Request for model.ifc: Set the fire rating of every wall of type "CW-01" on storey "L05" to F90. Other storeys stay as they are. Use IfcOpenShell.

First a look at what the model holds.

```python
import ifcopenshell
import ifcopenshell.util.element

model = ifcopenshell.open("model.ifc")
print(model.schema)
storey = next(s for s in model.by_type("IfcBuildingStorey") if s.Name == "L05")
walls = [e for e in ifcopenshell.util.element.get_decomposition(storey) if e.is_a("IfcWall")]
seen = {}
for e in walls:
    element_type = ifcopenshell.util.element.get_type(e)
    key = (element_type.Name if element_type != e and element_type else None, ifcopenshell.util.element.get_pset(e, "Pset_WallCommon", "FireRating"))
    seen[key] = seen.get(key, 0) + 1
for (name, value), count in sorted(seen.items(), key=str):
    print(count, "x", name, "|", value)
```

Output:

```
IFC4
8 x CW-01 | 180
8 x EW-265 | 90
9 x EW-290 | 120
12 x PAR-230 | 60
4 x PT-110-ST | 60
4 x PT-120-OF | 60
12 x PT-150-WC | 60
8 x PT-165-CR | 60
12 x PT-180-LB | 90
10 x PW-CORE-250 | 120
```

```python
import ifcopenshell
import ifcopenshell.api.pset
import ifcopenshell.util.element

model = ifcopenshell.open("model.ifc")

storey = next(s for s in model.by_type("IfcBuildingStorey") if s.Name == "L05")
walls = [e for e in ifcopenshell.util.element.get_decomposition(storey) if e.is_a("IfcWall")]

count = 0
for e in walls:
    element_type = ifcopenshell.util.element.get_type(e)
    if element_type in (None, e) or element_type.Name != "CW-01":
        continue
    # add_pset returns the element's existing set when there is one.
    pset = ifcopenshell.api.pset.add_pset(model, product=e, name="Pset_WallCommon")
    ifcopenshell.api.pset.edit_pset(model, pset=pset, properties={"FireRating": "F90"})
    count += 1

print(count, "walls updated")

model.write("model_rev.ifc")
```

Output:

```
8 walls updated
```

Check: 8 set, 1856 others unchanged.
